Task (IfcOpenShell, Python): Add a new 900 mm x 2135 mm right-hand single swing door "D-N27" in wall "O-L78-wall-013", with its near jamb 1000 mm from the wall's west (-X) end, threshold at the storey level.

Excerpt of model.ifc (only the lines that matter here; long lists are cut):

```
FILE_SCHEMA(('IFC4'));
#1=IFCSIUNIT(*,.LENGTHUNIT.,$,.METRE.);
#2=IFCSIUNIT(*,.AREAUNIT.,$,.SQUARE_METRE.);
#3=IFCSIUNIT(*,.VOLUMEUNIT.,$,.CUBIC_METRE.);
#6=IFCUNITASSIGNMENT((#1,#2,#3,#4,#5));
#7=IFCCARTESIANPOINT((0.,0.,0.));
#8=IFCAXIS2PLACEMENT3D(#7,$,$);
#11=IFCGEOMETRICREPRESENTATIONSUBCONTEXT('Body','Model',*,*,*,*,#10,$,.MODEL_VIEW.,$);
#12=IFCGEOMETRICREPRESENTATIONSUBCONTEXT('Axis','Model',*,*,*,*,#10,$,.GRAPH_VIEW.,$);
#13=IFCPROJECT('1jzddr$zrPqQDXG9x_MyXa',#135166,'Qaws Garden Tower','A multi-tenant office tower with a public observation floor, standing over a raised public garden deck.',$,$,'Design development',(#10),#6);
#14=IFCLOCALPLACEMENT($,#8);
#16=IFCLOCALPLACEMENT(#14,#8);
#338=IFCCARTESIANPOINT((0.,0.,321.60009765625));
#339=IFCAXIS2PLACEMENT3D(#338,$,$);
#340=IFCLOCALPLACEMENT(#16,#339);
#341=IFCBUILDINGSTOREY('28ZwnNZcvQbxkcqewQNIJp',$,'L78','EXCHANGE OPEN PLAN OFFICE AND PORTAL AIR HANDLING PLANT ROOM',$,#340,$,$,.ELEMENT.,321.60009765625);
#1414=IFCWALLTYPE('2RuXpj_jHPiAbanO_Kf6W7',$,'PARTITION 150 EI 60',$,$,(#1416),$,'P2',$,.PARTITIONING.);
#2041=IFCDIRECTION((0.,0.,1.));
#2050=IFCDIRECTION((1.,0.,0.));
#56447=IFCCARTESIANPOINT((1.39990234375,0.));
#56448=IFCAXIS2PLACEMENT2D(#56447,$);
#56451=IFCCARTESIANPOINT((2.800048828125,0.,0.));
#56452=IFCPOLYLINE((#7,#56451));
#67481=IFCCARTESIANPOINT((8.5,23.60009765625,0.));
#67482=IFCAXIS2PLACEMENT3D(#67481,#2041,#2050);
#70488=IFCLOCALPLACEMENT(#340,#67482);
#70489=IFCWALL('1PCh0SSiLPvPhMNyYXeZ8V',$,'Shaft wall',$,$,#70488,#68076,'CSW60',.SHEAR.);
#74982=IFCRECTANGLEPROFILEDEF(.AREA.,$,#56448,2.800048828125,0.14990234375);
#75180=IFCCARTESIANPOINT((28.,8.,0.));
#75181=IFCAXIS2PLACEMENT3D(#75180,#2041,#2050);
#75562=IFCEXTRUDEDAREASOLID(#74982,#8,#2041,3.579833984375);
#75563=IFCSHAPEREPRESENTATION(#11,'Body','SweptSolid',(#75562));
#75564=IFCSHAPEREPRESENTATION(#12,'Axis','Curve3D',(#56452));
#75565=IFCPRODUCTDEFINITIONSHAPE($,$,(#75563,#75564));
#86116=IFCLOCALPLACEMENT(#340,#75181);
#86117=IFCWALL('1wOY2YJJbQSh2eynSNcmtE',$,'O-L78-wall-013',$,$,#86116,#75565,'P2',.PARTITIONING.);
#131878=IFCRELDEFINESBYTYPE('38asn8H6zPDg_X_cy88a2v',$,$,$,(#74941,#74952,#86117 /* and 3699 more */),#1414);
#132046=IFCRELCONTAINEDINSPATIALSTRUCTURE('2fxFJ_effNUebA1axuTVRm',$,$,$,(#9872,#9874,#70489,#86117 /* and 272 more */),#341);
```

```python
import numpy as np
import ifcopenshell
import ifcopenshell.api.feature
import ifcopenshell.api.geometry
import ifcopenshell.api.root
import ifcopenshell.api.spatial
import ifcopenshell.geom
import ifcopenshell.util.element
import ifcopenshell.util.placement
import ifcopenshell.util.representation
import ifcopenshell.util.shape
import ifcopenshell.util.unit

model = ifcopenshell.open("model.ifc")
unit_scale = ifcopenshell.util.unit.calculate_unit_scale(model)
settings = ifcopenshell.geom.settings()


def volume(element):
    """Net volume in cubic metres, openings subtracted."""
    shape = ifcopenshell.geom.create_shape(settings, element)
    return ifcopenshell.util.shape.get_volume(shape.geometry)


wall = model.by_guid("1wOY2YJJbQSh2eynSNcmtE")
storey = ifcopenshell.util.element.get_container(wall, ifc_class="IfcBuildingStorey")
context = ifcopenshell.util.representation.get_context(model, "Model", "Body", "MODEL_VIEW")
before = volume(wall)

width, height, from_end, sill = 0.9, 2.135, 1, 0.0  # metres

# The wall runs along its own X axis, and the end named is its -X end.
wall_shape = ifcopenshell.geom.create_shape(settings, wall)
x, y, z = ifcopenshell.util.shape.get_vertices(wall_shape.geometry).T
start = x.min() + from_end
face, thickness = float(y.min()), float(y.max() - y.min())
wall_matrix = ifcopenshell.util.placement.get_local_placement(wall.ObjectPlacement)
level = ifcopenshell.util.placement.get_local_placement(storey.ObjectPlacement)[2, 3]


def in_wall(x, y):
    """Placement at x, y metres in the wall's axes, at sill height."""
    matrix = wall_matrix.copy()
    matrix[:, 3] = wall_matrix @ np.array([x / unit_scale, y / unit_scale, 0.0, 1.0])
    matrix[2, 3] = level + sill / unit_scale
    return matrix


# Opening: a box that overshoots both wall faces by 50 mm.
opening = ifcopenshell.api.root.create_entity(model, ifc_class="IfcOpeningElement", predefined_type="OPENING")
box = ifcopenshell.api.geometry.add_wall_representation(
    model, context=context, length=width, height=height, thickness=thickness + 0.1
)
ifcopenshell.api.geometry.assign_representation(model, product=opening, representation=box)
ifcopenshell.api.geometry.edit_object_placement(model, product=opening, matrix=in_wall(start, face - 0.05), is_si=False)
ifcopenshell.api.feature.add_feature(model, feature=opening, element=wall)

door = ifcopenshell.api.root.create_entity(model, ifc_class="IfcDoor", name="D-N27", predefined_type="DOOR")
door.OverallWidth, door.OverallHeight = width / unit_scale, height / unit_scale
door.OperationType = "SINGLE_SWING_RIGHT"
body = ifcopenshell.api.geometry.add_door_representation(
    model,
    context=context,
    overall_width=door.OverallWidth,
    overall_height=door.OverallHeight,
    operation_type="SINGLE_SWING_RIGHT",
    lining_properties={"LiningDepth": thickness / unit_scale, "ThresholdDepth": thickness / unit_scale},
)
ifcopenshell.api.geometry.assign_representation(model, product=door, representation=body)
ifcopenshell.api.spatial.assign_container(model, products=[door], relating_structure=storey)
ifcopenshell.api.feature.add_filling(model, opening=opening, element=door)

# The lining spans the wall, so the door starts at the wall face.
ifcopenshell.api.geometry.edit_object_placement(model, product=door, matrix=in_wall(start, face), is_si=False)

after = volume(wall)

print(f"wall volume {before:.3f} -> {after:.3f} m3")

model.write("model_updated.ifc")
```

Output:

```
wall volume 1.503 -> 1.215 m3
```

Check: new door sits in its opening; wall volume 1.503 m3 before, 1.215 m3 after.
